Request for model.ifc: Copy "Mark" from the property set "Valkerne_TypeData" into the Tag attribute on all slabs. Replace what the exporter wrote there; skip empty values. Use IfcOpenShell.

First a look at what the model holds.

```python
import ifcopenshell
import ifcopenshell.util.element

model = ifcopenshell.open("model.ifc")
print(model.schema)
slabs = model.by_type("IfcSlab")
print(len(slabs), "slabs")
for e in slabs[:8]:
    source = ifcopenshell.util.element.get_pset(e, "Valkerne_TypeData", "Mark")
    target = e.Tag
    print(e.id(), repr(source), repr(target), sep=" | ")
```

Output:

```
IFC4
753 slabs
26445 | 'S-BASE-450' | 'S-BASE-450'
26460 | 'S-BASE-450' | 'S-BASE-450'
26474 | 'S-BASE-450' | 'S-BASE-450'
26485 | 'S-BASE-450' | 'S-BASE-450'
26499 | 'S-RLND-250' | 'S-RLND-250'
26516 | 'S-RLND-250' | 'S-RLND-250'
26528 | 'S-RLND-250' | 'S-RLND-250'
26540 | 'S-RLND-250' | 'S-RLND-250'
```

```python
import ifcopenshell
import ifcopenshell.util.element

model = ifcopenshell.open("model.ifc")

count = 0
for e in model.by_type("IfcSlab"):
    value = ifcopenshell.util.element.get_pset(e, "Valkerne_TypeData", "Mark")
    current = e.Tag
    if not value or not value.strip() or current == value:
        continue
    e.Tag = value
    count += 1

print(count, "slabs updated")

model.write("model_rev.ifc")
```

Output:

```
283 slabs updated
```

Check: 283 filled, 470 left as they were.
